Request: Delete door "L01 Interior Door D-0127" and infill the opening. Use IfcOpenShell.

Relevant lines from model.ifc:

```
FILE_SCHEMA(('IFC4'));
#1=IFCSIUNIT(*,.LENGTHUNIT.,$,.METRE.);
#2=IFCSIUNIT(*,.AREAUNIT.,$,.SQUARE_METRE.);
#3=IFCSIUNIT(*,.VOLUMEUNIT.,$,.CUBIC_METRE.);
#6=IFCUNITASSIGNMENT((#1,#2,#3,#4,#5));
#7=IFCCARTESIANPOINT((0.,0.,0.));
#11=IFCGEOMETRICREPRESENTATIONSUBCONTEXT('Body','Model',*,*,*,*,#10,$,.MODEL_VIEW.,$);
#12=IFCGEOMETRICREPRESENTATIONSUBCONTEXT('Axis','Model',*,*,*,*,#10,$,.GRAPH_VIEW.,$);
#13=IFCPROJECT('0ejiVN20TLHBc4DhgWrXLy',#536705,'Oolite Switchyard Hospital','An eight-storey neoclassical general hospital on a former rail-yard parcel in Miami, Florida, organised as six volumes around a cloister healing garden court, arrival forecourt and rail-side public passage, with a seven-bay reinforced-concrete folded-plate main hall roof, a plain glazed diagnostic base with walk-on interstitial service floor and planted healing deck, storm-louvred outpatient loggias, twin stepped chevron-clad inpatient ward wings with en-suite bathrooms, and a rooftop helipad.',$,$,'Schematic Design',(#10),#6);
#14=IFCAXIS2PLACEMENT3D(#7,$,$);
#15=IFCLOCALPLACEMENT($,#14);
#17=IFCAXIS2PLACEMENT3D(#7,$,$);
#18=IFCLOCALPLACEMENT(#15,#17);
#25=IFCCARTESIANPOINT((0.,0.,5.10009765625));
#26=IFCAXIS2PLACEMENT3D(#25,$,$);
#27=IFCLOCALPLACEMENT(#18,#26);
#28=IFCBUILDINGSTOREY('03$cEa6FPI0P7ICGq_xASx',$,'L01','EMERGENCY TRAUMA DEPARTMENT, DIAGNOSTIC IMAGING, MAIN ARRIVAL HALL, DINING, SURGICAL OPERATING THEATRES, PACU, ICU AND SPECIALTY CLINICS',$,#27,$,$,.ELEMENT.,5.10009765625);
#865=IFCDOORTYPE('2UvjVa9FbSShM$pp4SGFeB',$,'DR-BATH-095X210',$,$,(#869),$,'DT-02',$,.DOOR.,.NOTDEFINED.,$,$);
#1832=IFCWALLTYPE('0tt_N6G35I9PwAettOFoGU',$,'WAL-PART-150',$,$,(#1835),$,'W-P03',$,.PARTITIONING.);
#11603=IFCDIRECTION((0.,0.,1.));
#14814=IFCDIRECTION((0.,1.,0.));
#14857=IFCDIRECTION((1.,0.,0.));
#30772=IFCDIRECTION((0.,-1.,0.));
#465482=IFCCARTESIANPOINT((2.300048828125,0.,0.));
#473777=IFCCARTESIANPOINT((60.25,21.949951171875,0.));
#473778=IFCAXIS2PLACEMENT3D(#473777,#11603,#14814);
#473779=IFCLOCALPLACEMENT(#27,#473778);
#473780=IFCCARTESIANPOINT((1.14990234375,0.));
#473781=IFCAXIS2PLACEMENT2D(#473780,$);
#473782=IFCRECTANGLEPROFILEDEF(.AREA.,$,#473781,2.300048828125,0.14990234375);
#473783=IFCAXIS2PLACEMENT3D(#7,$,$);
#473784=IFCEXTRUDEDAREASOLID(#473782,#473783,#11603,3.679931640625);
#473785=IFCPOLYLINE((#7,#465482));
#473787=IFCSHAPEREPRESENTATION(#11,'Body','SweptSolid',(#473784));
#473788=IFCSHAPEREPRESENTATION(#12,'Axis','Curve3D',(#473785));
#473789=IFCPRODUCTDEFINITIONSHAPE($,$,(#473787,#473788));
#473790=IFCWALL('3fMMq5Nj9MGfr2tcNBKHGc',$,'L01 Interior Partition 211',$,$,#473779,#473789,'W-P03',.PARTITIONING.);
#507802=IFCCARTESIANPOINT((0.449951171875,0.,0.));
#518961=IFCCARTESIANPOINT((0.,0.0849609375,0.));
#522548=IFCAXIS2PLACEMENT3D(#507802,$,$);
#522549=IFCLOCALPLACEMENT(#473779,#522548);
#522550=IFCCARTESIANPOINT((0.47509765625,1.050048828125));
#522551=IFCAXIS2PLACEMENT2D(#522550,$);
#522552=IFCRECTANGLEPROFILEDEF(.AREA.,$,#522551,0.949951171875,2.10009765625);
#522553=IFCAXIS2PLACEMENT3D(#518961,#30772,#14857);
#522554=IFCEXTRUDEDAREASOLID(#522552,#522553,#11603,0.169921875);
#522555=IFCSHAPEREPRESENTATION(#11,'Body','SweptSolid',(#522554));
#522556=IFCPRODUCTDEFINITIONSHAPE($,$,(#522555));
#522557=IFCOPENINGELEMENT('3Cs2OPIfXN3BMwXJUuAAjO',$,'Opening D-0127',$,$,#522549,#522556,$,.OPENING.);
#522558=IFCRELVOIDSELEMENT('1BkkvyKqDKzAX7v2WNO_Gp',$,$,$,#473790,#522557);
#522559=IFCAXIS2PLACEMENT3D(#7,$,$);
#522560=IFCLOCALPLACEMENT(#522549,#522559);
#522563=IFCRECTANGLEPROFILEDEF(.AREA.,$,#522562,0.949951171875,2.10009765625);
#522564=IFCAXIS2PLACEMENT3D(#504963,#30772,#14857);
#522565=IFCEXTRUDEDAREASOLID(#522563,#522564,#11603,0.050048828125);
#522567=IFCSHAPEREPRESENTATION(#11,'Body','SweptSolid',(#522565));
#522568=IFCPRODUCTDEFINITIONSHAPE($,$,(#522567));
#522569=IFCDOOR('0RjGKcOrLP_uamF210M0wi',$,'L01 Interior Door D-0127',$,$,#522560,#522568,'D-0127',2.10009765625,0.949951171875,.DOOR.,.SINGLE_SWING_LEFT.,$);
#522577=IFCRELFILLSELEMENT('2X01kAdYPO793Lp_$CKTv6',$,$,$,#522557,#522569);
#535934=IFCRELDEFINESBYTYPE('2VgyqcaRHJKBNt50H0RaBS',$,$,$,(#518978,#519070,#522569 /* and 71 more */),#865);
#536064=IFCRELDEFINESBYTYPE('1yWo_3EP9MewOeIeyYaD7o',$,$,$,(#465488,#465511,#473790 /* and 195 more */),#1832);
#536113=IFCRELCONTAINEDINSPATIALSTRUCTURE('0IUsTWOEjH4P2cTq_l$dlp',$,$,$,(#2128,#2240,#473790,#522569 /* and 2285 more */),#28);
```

```python
import ifcopenshell
import ifcopenshell.api.feature
import ifcopenshell.api.root
import ifcopenshell.geom
import ifcopenshell.util.shape

model = ifcopenshell.open("model.ifc")
settings = ifcopenshell.geom.settings()


def volume(element):
    """Net volume in cubic metres, openings subtracted."""
    shape = ifcopenshell.geom.create_shape(settings, element)
    return ifcopenshell.util.shape.get_volume(shape.geometry)


door = model.by_guid("0RjGKcOrLP_uamF210M0wi")
opening = door.FillsVoids[0].RelatingOpeningElement
wall = opening.VoidsElements[0].RelatingBuildingElement
before = volume(wall)

ifcopenshell.api.root.remove_product(model, product=door)
ifcopenshell.api.feature.remove_feature(model, feature=opening)

after = volume(wall)

print(f"wall volume {before:.3f} -> {after:.3f} m3")

model.write("model_rev.ifc")
```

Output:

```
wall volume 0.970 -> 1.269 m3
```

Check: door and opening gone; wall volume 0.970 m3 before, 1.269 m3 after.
